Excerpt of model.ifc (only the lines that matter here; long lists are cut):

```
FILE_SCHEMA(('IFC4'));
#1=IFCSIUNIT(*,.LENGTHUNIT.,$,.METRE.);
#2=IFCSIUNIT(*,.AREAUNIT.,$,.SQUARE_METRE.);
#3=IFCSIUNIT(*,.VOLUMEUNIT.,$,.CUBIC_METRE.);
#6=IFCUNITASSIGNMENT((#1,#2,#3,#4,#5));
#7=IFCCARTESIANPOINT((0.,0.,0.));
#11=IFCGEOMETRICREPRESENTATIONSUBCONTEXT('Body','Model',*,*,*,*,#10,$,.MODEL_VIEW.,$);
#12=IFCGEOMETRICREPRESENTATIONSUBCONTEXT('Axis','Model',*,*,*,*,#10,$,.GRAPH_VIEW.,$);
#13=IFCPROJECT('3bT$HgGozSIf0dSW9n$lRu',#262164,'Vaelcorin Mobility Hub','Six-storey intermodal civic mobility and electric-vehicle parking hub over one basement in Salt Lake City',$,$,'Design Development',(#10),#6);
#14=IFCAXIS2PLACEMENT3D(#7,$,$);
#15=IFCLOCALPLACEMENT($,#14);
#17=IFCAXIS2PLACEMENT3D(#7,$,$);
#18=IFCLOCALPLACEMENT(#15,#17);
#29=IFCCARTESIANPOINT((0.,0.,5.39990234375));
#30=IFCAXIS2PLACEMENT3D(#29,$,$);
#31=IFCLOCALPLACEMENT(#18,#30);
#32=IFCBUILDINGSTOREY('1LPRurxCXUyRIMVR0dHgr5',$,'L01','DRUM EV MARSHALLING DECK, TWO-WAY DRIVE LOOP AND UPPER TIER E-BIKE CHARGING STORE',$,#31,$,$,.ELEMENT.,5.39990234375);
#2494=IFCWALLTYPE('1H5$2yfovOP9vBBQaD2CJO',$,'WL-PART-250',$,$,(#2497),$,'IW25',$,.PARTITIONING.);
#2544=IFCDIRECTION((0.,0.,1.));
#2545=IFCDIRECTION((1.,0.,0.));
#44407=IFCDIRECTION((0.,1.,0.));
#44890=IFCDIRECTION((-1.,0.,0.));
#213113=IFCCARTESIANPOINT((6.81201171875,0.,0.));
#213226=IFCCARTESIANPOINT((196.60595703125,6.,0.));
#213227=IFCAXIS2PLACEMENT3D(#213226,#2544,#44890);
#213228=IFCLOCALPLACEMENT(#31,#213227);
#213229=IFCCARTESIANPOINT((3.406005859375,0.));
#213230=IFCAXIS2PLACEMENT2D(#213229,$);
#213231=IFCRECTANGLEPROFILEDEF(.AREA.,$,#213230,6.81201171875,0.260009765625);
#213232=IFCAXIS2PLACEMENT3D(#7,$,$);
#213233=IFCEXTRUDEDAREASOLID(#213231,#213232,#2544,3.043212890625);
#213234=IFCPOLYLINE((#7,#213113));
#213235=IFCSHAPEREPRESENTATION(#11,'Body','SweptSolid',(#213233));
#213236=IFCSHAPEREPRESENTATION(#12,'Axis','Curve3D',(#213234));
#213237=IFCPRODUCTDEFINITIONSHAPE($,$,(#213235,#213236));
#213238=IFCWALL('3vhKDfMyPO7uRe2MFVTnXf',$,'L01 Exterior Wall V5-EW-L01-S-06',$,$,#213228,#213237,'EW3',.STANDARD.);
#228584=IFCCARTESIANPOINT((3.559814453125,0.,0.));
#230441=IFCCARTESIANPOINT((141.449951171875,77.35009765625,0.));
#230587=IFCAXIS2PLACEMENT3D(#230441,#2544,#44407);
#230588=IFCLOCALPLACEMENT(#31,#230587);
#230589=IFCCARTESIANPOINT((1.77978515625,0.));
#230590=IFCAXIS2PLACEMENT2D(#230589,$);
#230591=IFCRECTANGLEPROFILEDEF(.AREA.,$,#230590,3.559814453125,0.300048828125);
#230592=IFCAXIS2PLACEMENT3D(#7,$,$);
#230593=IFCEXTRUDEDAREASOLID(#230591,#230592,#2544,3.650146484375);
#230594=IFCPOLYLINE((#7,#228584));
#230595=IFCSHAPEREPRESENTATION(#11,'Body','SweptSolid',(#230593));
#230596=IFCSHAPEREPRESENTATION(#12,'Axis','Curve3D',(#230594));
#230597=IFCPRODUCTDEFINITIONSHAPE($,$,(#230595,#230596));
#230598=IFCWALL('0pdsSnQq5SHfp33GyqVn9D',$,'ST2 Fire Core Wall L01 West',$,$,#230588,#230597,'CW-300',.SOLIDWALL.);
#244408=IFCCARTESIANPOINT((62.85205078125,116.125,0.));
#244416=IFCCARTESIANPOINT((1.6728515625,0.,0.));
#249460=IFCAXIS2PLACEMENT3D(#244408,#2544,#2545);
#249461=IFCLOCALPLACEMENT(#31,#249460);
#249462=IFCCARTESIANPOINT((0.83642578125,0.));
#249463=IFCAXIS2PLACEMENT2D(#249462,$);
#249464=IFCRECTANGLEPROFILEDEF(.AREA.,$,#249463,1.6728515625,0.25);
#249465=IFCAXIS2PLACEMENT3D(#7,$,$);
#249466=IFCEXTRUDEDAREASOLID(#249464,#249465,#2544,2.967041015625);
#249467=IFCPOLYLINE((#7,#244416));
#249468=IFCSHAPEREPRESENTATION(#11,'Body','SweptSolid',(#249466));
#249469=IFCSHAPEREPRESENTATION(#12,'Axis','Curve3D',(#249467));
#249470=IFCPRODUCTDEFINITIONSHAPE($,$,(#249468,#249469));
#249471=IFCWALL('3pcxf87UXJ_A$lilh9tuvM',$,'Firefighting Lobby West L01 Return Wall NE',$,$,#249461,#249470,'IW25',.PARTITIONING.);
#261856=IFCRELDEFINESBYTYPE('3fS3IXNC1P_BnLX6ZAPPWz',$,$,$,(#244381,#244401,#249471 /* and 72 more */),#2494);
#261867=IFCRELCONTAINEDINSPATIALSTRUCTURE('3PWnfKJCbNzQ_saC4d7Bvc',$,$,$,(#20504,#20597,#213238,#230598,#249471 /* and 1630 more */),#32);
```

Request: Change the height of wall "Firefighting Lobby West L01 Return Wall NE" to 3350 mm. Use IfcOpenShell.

```python
import ifcopenshell
import ifcopenshell.geom
import ifcopenshell.util.representation
import ifcopenshell.util.shape
import ifcopenshell.util.unit

model = ifcopenshell.open("model.ifc")
unit_scale = ifcopenshell.util.unit.calculate_unit_scale(model)
settings = ifcopenshell.geom.settings()


def volume(element):
    """Net volume in cubic metres, openings subtracted."""
    shape = ifcopenshell.geom.create_shape(settings, element)
    return ifcopenshell.util.shape.get_volume(shape.geometry)


wall = model.by_guid("3pcxf87UXJ_A$lilh9tuvM")
before = volume(wall)

body = ifcopenshell.util.representation.get_representation(wall, "Model", "Body")
solid = body.Items[0]
old_height = solid.Depth
solid.Depth = 3.35 / unit_scale
after = volume(wall)

print(f"height {old_height:g} -> {solid.Depth:g}, volume {before:.3f} -> {after:.3f} m3")

model.write("model_v2.ifc")
```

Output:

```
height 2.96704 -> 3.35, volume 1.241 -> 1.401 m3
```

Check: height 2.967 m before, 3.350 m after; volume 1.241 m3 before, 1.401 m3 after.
